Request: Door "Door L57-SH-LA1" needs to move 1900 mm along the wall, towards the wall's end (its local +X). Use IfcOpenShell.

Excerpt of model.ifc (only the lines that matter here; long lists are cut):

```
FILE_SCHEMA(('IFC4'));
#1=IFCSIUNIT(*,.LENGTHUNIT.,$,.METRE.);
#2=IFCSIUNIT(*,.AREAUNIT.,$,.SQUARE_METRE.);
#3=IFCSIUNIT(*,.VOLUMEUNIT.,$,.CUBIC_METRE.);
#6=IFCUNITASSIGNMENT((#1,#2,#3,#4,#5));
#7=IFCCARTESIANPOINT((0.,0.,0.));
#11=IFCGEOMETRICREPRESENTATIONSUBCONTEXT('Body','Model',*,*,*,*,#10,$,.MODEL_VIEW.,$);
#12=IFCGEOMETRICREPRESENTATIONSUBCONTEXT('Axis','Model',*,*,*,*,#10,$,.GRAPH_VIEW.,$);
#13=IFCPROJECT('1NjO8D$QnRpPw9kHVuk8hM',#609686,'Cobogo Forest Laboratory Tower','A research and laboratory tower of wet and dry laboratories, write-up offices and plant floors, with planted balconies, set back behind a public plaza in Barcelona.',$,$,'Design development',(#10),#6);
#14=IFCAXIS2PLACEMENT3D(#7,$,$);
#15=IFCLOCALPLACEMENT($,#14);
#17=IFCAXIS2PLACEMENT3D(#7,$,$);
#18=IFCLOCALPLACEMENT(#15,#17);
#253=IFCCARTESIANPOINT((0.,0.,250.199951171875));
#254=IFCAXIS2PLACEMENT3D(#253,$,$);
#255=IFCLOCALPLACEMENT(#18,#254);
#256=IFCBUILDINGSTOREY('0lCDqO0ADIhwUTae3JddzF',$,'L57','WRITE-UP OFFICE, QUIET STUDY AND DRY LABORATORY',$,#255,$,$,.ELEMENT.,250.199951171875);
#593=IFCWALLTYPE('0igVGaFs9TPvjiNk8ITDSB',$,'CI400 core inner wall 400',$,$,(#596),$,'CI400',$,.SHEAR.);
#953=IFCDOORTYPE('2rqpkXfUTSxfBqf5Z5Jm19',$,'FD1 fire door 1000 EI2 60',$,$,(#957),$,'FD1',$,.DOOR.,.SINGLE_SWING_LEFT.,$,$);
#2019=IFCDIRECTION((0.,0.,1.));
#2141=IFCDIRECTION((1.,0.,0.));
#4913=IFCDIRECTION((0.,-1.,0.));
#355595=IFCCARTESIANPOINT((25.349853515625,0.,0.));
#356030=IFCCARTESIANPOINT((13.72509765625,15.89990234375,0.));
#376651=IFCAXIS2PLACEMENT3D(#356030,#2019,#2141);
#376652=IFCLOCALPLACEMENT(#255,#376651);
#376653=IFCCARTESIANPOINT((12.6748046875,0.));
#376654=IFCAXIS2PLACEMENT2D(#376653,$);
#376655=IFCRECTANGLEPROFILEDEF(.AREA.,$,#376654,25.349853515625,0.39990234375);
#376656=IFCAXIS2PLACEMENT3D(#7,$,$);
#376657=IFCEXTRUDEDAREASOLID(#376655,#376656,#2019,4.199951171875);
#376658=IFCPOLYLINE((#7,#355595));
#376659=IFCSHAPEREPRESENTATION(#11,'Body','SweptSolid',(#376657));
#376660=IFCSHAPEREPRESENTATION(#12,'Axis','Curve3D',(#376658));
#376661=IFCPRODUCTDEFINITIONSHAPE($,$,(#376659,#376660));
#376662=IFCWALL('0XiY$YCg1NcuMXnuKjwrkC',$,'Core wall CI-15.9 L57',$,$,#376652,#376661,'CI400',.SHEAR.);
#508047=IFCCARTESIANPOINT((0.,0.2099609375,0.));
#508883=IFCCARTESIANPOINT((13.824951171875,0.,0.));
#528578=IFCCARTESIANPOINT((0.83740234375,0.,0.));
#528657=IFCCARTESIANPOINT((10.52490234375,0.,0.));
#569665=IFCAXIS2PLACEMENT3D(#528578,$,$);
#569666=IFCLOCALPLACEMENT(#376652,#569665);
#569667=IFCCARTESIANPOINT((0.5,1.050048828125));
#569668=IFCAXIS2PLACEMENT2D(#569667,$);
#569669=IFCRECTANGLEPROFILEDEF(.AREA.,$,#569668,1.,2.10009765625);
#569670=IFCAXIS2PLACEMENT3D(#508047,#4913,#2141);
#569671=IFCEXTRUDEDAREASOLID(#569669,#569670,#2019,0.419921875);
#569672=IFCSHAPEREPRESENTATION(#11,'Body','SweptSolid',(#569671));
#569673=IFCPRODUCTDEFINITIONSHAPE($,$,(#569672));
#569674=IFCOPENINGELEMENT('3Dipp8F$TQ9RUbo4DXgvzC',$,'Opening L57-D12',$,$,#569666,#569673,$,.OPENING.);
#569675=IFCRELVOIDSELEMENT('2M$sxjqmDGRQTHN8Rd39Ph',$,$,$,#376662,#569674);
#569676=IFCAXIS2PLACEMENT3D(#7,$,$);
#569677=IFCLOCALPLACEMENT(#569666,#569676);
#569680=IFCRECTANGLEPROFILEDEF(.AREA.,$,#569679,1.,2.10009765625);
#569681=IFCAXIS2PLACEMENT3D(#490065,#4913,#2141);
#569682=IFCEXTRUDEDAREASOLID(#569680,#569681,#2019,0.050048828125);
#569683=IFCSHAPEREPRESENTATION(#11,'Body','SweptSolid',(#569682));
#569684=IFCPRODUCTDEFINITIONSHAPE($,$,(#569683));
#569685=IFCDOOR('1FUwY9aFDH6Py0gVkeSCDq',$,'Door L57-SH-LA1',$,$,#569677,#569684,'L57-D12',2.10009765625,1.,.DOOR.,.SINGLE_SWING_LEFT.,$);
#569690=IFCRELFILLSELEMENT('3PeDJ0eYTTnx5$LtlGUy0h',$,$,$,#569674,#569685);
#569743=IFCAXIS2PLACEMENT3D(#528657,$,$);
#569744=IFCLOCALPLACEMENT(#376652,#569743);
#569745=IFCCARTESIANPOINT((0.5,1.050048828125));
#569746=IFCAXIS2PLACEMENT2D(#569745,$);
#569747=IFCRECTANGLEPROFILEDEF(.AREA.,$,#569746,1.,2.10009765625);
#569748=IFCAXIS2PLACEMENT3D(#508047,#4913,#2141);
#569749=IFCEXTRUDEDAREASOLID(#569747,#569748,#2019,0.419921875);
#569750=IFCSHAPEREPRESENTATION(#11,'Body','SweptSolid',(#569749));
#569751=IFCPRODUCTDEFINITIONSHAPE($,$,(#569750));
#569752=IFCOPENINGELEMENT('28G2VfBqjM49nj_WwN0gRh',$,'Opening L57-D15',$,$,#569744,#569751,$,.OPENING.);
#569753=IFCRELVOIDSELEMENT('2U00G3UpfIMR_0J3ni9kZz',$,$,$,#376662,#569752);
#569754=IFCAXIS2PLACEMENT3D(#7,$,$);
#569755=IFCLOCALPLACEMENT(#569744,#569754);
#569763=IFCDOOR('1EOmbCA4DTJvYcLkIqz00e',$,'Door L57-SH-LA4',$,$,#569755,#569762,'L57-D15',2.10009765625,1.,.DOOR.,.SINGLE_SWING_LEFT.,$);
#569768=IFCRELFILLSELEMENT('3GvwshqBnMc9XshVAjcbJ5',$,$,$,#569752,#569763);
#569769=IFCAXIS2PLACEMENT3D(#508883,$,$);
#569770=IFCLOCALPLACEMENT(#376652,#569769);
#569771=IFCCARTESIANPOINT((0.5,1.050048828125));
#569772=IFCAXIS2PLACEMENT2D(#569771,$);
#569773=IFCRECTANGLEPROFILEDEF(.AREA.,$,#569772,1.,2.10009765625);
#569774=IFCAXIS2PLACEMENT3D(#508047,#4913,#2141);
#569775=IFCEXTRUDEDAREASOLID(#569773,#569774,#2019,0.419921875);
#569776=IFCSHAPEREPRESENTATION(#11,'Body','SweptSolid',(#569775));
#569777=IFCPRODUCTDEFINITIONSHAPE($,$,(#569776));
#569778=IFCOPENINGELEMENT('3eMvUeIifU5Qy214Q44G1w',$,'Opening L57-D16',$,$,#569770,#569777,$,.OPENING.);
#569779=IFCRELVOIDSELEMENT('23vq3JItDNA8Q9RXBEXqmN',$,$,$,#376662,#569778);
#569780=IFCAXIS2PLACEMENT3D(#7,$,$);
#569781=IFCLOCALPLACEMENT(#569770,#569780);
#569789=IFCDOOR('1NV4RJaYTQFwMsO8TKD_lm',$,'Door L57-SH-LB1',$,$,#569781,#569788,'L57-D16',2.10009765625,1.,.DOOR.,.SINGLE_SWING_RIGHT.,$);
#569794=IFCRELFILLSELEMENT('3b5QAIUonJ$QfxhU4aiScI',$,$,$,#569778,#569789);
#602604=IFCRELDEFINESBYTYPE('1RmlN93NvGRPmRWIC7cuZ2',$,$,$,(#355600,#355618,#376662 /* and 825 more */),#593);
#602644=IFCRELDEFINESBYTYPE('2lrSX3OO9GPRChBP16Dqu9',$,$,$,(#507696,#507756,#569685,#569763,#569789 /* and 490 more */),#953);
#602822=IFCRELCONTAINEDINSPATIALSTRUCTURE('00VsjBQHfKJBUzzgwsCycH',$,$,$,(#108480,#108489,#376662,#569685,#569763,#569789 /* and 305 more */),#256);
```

```python
import ifcopenshell
import ifcopenshell.api.geometry
import ifcopenshell.util.placement

model = ifcopenshell.open("model.ifc")

door = model.by_guid("1FUwY9aFDH6Py0gVkeSCDq")
opening = door.FillsVoids[0].RelatingOpeningElement
wall = opening.VoidsElements[0].RelatingBuildingElement

wall_matrix = ifcopenshell.util.placement.get_local_placement(wall.ObjectPlacement)
shift = wall_matrix[:3, 0] * 1.9
before = ifcopenshell.util.placement.get_local_placement(door.ObjectPlacement)[:3, 3].copy()

# The door is placed relative to its opening, so it follows when the opening moves.
matrix = ifcopenshell.util.placement.get_local_placement(opening.ObjectPlacement)
matrix[:3, 3] += shift
ifcopenshell.api.geometry.edit_object_placement(
    model, product=opening, matrix=matrix, is_si=False, should_transform_children=True
)

after = ifcopenshell.util.placement.get_local_placement(door.ObjectPlacement)[:3, 3]
print("door moved by", (after - before).round(3) + 0.0)

model.write("model_updated.ifc")
```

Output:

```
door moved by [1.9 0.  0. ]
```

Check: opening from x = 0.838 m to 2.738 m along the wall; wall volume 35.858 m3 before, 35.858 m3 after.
